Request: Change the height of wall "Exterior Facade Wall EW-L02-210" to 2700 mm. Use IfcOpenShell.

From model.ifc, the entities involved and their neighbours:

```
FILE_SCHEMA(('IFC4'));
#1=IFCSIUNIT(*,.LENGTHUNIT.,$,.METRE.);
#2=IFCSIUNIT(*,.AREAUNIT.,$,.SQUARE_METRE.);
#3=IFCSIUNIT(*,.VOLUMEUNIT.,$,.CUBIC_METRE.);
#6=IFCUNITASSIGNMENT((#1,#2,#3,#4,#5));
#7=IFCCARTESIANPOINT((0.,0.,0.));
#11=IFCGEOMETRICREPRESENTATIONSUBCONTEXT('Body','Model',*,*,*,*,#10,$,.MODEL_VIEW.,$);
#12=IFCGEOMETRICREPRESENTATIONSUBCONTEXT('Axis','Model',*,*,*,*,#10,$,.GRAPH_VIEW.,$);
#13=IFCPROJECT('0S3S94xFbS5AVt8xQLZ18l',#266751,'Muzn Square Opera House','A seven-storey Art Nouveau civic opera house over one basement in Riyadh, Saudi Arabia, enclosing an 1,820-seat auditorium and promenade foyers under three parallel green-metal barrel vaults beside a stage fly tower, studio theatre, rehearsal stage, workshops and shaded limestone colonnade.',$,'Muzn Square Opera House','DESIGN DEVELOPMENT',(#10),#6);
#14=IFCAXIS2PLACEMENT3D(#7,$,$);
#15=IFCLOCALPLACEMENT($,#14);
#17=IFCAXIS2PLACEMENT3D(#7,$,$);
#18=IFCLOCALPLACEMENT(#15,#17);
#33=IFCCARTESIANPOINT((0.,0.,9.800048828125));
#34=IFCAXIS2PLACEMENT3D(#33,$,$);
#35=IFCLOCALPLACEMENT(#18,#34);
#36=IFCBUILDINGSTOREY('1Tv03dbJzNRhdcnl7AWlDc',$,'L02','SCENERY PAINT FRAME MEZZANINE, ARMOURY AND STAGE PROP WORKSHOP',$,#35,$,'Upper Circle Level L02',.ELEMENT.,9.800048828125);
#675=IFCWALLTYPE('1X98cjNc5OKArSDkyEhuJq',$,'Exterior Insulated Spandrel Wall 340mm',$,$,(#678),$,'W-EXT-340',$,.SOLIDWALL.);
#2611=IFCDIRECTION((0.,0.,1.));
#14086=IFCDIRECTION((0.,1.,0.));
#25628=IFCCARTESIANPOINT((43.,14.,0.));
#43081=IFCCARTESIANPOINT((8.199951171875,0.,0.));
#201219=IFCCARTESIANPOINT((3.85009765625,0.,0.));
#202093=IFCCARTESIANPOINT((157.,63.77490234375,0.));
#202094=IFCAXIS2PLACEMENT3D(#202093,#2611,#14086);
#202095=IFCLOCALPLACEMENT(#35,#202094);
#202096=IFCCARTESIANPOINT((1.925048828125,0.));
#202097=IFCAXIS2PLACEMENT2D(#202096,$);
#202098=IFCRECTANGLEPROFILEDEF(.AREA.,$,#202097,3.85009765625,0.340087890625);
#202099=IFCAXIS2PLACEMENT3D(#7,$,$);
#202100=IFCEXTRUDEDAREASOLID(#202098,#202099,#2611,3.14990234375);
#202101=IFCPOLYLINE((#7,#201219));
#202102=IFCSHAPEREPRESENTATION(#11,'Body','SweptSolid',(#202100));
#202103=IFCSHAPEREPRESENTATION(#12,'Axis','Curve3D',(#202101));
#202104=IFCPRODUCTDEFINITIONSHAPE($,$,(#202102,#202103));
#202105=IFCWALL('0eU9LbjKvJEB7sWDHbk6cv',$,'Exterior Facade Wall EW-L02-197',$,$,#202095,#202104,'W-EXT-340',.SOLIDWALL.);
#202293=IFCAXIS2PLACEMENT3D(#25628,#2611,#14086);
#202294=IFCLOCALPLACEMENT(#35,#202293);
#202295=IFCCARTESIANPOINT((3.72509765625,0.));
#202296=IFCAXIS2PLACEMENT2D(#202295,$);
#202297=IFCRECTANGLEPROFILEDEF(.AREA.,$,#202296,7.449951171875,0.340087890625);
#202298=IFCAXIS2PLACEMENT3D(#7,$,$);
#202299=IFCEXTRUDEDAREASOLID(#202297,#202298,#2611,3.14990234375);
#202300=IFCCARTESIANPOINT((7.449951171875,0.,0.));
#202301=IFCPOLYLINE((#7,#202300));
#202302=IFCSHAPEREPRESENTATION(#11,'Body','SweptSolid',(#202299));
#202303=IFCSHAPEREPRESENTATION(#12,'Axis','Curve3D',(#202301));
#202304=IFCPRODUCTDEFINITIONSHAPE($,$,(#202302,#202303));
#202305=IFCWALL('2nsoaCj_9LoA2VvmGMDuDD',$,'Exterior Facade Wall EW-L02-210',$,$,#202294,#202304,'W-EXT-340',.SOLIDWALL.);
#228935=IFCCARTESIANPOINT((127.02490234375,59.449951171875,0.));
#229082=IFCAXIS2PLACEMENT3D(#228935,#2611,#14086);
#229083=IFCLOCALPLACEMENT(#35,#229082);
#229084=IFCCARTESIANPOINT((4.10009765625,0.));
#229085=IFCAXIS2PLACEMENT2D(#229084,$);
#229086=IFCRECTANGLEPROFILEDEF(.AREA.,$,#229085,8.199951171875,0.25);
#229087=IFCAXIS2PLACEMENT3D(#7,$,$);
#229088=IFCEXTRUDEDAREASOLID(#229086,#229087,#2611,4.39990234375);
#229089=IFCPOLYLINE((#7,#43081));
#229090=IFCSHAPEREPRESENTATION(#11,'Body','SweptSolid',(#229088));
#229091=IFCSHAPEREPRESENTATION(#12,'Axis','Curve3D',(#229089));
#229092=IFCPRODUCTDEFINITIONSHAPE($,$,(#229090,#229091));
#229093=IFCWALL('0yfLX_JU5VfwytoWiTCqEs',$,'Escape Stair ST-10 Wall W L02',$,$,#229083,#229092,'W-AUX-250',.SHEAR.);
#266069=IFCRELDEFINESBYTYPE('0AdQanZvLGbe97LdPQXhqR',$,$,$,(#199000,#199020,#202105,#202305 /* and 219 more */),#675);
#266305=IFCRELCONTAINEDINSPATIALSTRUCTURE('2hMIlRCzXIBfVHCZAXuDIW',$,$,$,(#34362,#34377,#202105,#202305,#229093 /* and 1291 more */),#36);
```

```python
import ifcopenshell
import ifcopenshell.geom
import ifcopenshell.util.representation
import ifcopenshell.util.shape
import ifcopenshell.util.unit

model = ifcopenshell.open("model.ifc")
unit_scale = ifcopenshell.util.unit.calculate_unit_scale(model)
settings = ifcopenshell.geom.settings()


def volume(element):
    """Net volume in cubic metres, openings subtracted."""
    shape = ifcopenshell.geom.create_shape(settings, element)
    return ifcopenshell.util.shape.get_volume(shape.geometry)


wall = model.by_guid("2nsoaCj_9LoA2VvmGMDuDD")
before = volume(wall)

body = ifcopenshell.util.representation.get_representation(wall, "Model", "Body")
solid = body.Items[0]
old_height = solid.Depth
solid.Depth = 2.7 / unit_scale
after = volume(wall)

print(f"height {old_height:g} -> {solid.Depth:g}, volume {before:.3f} -> {after:.3f} m3")

model.write("model-out.ifc")
```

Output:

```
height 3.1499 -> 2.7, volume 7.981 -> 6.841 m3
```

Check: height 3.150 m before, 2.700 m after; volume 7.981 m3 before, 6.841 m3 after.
